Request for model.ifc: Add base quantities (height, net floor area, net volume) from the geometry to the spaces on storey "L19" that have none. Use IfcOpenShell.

First a look at what the model holds.

```python
import ifcopenshell
import ifcopenshell.util.element
import ifcopenshell.util.unit

model = ifcopenshell.open("model.ifc")
print(model.schema)
for unit_type in ("LENGTHUNIT", "AREAUNIT", "VOLUMEUNIT"):
    print(unit_type, ifcopenshell.util.unit.calculate_unit_scale(model, unit_type))
storey = next(s for s in model.by_type("IfcBuildingStorey") if s.Name == "L19")
spaces = [e for e in ifcopenshell.util.element.get_decomposition(storey) if e.is_a("IfcSpace")]
for e in sorted(spaces, key=lambda e: e.id()):
    print(e.id(), e.is_a(), e.Name, list(ifcopenshell.util.element.get_psets(e, qtos_only=True)), sep=" | ")
```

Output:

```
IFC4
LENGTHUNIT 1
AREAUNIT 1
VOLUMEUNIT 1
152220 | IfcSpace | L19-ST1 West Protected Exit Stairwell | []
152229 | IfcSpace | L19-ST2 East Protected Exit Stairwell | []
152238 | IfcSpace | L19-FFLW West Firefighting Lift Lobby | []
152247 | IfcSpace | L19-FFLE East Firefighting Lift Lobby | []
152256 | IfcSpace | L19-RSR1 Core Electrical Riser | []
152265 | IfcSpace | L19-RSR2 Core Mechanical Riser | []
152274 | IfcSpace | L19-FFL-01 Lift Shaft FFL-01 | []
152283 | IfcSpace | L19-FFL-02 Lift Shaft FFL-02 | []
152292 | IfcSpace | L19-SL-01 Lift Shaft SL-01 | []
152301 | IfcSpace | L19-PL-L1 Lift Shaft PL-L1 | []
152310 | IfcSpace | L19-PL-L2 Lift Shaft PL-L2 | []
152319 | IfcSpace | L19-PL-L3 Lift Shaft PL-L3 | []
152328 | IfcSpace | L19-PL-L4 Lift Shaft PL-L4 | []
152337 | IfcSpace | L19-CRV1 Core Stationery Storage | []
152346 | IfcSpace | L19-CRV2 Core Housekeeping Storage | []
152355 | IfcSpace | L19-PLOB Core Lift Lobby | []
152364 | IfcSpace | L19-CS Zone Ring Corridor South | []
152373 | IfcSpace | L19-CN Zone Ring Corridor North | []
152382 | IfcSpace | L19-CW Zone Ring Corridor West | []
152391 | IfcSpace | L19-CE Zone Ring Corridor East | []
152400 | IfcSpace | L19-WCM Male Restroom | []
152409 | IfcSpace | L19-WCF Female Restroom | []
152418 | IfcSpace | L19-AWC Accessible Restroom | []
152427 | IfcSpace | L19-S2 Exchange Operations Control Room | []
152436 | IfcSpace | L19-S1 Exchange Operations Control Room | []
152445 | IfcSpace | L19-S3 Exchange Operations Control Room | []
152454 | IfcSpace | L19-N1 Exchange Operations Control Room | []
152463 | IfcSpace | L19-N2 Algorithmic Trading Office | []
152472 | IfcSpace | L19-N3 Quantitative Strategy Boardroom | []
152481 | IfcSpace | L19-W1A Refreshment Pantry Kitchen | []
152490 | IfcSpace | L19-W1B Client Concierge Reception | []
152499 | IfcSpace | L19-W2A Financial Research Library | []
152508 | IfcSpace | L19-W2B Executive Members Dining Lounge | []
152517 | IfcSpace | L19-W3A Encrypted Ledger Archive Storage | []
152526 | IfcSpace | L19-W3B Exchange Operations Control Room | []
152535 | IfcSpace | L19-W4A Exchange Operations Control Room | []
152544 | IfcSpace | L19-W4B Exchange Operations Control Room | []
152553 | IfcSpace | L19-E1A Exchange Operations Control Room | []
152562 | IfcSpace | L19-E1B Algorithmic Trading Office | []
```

```python
import ifcopenshell
import ifcopenshell.api.pset
import ifcopenshell.geom
import ifcopenshell.util.element
import ifcopenshell.util.shape
import ifcopenshell.util.unit

model = ifcopenshell.open("model.ifc")
unit_scale = ifcopenshell.util.unit.calculate_unit_scale(model)
area_scale = ifcopenshell.util.unit.calculate_unit_scale(model, "AREAUNIT")
volume_scale = ifcopenshell.util.unit.calculate_unit_scale(model, "VOLUMEUNIT")
settings = ifcopenshell.geom.settings()

storey = next(s for s in model.by_type("IfcBuildingStorey") if s.Name == "L19")
spaces = [e for e in ifcopenshell.util.element.get_decomposition(storey) if e.is_a("IfcSpace")]

for e in sorted(spaces, key=lambda e: e.id()):
    if ifcopenshell.util.element.get_psets(e, qtos_only=True, should_inherit=False):
        continue
    # Geometry comes back in metres, in the element's own axes.
    shape = ifcopenshell.geom.create_shape(settings, e)
    values = {
        "Height": ifcopenshell.util.shape.get_z(shape.geometry) / unit_scale,
        "NetFloorArea": ifcopenshell.util.shape.get_footprint_area(shape.geometry) / area_scale,
        "NetVolume": ifcopenshell.util.shape.get_volume(shape.geometry) / volume_scale,
    }
    qto = ifcopenshell.api.pset.add_qto(model, product=e, name="Qto_SpaceBaseQuantities")
    ifcopenshell.api.pset.edit_qto(model, qto=qto, properties=values)
    print(e.id(), {k: round(v, 3) for k, v in values.items()})

model.write("model_rev.ifc")
```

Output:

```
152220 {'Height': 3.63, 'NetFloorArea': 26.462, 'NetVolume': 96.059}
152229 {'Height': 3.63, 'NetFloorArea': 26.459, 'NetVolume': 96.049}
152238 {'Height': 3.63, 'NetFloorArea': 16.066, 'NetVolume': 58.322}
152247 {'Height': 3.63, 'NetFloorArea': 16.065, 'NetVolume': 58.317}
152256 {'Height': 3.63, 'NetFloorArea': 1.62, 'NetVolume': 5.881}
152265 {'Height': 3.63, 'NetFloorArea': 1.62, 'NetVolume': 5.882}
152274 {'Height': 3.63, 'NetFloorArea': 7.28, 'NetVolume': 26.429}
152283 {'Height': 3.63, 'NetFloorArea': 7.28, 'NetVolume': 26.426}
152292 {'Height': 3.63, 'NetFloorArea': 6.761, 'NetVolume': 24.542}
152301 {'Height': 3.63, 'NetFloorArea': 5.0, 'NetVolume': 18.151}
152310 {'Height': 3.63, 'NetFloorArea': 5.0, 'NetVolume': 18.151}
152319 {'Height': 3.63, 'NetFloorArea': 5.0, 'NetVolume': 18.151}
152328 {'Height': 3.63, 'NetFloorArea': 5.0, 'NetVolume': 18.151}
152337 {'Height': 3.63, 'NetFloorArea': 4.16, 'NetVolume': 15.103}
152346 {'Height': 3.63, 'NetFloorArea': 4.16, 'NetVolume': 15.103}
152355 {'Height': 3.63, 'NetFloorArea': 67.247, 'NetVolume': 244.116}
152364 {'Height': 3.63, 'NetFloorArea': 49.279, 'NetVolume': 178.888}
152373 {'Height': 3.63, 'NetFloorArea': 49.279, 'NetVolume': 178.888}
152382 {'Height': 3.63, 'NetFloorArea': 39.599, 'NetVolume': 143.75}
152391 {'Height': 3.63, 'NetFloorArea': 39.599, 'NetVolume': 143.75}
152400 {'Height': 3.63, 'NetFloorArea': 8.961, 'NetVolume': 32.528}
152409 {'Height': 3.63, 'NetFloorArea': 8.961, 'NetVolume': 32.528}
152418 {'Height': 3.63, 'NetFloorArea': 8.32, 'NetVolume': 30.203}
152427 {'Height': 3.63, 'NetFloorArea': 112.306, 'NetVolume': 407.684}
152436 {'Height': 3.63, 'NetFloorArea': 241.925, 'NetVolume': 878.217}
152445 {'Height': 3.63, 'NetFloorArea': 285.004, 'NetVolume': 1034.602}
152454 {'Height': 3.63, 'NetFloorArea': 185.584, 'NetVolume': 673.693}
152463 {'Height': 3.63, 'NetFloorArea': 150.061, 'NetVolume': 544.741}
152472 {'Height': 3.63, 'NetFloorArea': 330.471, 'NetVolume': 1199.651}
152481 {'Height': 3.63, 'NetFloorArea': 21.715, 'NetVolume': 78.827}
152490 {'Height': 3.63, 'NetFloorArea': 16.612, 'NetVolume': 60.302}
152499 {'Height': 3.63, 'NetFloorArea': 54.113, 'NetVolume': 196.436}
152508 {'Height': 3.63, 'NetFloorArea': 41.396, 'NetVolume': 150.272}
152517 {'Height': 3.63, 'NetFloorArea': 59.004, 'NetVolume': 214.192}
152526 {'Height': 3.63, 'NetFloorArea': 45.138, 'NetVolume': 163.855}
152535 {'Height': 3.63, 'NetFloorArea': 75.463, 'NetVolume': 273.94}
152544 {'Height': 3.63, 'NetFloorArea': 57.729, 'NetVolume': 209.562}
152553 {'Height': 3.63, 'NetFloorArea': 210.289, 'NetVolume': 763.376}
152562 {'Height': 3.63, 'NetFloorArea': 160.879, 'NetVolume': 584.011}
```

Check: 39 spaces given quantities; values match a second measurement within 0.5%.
